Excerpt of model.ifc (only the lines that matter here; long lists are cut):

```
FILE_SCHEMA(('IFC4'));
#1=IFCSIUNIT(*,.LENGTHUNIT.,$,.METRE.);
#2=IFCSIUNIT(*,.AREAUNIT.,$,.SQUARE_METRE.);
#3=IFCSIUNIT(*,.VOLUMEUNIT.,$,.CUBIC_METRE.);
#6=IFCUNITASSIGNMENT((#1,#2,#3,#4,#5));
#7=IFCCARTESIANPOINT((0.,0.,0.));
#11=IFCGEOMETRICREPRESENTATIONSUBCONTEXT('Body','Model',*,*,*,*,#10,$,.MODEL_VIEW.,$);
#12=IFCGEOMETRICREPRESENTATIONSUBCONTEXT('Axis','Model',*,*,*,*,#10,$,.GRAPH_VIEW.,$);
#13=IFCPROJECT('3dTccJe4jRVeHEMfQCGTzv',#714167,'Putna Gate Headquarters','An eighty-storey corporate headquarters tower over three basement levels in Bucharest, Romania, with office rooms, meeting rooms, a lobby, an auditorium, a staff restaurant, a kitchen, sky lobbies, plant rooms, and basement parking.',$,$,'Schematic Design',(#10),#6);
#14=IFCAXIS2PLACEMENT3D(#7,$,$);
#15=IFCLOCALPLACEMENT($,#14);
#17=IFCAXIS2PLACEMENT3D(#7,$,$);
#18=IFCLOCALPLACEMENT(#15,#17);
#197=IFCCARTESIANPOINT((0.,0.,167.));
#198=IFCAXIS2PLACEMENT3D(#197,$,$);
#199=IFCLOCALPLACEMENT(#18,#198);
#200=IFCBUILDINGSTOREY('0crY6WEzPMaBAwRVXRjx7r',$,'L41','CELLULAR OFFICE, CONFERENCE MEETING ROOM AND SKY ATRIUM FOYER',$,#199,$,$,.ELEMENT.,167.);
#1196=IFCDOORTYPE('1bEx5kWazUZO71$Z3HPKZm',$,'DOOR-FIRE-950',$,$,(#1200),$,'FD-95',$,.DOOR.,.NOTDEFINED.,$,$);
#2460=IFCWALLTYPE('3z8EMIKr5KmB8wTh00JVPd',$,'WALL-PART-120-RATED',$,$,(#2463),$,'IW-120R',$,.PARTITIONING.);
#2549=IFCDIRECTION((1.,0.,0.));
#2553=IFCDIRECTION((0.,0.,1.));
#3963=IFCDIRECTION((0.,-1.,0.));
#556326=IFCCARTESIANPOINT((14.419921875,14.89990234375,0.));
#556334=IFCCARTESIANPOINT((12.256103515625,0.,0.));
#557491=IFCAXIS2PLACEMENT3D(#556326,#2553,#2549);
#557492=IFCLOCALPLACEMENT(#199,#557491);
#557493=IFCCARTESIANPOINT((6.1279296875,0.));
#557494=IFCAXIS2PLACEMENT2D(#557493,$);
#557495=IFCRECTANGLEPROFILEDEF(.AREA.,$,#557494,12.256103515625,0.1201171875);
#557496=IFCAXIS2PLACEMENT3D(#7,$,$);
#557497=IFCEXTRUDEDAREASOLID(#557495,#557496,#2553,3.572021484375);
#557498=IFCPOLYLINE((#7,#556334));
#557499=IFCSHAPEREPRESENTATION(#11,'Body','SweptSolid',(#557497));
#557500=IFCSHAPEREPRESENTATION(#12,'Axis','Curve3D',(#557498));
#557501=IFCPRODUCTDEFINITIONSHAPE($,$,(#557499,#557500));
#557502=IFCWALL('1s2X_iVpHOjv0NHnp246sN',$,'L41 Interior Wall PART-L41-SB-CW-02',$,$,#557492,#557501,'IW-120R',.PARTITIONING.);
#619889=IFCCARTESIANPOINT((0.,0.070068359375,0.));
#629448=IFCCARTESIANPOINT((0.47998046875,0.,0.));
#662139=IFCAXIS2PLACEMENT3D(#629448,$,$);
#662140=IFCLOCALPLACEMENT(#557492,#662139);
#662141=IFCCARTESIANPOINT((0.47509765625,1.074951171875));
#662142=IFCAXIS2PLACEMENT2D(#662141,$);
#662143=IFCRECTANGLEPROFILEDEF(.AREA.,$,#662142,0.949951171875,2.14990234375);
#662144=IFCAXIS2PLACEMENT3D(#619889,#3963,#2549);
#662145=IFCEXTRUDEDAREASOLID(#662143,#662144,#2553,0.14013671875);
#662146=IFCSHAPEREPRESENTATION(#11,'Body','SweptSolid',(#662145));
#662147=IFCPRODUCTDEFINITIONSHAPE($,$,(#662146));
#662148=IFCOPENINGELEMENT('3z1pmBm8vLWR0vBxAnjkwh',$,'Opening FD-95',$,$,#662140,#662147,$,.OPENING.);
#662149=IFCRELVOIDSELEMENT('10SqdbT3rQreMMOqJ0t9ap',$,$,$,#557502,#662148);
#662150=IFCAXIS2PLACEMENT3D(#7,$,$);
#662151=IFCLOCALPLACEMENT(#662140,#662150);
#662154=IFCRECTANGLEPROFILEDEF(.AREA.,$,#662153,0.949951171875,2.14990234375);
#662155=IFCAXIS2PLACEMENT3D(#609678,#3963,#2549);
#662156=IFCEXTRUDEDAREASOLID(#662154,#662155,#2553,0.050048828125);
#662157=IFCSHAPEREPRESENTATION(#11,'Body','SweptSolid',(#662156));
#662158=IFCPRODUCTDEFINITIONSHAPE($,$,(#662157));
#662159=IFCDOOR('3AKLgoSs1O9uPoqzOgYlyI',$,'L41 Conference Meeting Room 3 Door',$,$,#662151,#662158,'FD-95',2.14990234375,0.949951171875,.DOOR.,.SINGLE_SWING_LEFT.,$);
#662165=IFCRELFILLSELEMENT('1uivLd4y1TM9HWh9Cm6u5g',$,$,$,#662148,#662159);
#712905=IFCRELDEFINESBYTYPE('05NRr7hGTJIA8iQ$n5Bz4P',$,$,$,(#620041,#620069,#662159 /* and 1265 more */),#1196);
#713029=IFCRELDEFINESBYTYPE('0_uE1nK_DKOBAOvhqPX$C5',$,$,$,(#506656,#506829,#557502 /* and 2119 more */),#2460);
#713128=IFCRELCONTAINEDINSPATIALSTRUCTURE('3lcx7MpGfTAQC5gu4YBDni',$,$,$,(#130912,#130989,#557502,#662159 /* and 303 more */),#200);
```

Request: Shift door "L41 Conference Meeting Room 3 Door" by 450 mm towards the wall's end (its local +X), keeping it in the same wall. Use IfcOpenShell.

```python
import ifcopenshell
import ifcopenshell.api.geometry
import ifcopenshell.util.placement
import ifcopenshell.util.unit

model = ifcopenshell.open("model.ifc")
unit_scale = ifcopenshell.util.unit.calculate_unit_scale(model)

door = model.by_guid("3AKLgoSs1O9uPoqzOgYlyI")
opening = door.FillsVoids[0].RelatingOpeningElement
wall = opening.VoidsElements[0].RelatingBuildingElement

wall_matrix = ifcopenshell.util.placement.get_local_placement(wall.ObjectPlacement)
shift = wall_matrix[:3, 0] * 0.45 / unit_scale
before = ifcopenshell.util.placement.get_local_placement(door.ObjectPlacement)[:3, 3].copy()

# The door is placed relative to its opening, so it follows when the opening moves.
matrix = ifcopenshell.util.placement.get_local_placement(opening.ObjectPlacement)
matrix[:3, 3] += shift
ifcopenshell.api.geometry.edit_object_placement(
    model, product=opening, matrix=matrix, is_si=False, should_transform_children=True
)

after = ifcopenshell.util.placement.get_local_placement(door.ObjectPlacement)[:3, 3]
print("door moved by", (after - before).round(3) + 0.0)

model.write("model_updated.ifc")
```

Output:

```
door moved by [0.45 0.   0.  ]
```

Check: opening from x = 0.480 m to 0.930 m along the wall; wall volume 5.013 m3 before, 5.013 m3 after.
